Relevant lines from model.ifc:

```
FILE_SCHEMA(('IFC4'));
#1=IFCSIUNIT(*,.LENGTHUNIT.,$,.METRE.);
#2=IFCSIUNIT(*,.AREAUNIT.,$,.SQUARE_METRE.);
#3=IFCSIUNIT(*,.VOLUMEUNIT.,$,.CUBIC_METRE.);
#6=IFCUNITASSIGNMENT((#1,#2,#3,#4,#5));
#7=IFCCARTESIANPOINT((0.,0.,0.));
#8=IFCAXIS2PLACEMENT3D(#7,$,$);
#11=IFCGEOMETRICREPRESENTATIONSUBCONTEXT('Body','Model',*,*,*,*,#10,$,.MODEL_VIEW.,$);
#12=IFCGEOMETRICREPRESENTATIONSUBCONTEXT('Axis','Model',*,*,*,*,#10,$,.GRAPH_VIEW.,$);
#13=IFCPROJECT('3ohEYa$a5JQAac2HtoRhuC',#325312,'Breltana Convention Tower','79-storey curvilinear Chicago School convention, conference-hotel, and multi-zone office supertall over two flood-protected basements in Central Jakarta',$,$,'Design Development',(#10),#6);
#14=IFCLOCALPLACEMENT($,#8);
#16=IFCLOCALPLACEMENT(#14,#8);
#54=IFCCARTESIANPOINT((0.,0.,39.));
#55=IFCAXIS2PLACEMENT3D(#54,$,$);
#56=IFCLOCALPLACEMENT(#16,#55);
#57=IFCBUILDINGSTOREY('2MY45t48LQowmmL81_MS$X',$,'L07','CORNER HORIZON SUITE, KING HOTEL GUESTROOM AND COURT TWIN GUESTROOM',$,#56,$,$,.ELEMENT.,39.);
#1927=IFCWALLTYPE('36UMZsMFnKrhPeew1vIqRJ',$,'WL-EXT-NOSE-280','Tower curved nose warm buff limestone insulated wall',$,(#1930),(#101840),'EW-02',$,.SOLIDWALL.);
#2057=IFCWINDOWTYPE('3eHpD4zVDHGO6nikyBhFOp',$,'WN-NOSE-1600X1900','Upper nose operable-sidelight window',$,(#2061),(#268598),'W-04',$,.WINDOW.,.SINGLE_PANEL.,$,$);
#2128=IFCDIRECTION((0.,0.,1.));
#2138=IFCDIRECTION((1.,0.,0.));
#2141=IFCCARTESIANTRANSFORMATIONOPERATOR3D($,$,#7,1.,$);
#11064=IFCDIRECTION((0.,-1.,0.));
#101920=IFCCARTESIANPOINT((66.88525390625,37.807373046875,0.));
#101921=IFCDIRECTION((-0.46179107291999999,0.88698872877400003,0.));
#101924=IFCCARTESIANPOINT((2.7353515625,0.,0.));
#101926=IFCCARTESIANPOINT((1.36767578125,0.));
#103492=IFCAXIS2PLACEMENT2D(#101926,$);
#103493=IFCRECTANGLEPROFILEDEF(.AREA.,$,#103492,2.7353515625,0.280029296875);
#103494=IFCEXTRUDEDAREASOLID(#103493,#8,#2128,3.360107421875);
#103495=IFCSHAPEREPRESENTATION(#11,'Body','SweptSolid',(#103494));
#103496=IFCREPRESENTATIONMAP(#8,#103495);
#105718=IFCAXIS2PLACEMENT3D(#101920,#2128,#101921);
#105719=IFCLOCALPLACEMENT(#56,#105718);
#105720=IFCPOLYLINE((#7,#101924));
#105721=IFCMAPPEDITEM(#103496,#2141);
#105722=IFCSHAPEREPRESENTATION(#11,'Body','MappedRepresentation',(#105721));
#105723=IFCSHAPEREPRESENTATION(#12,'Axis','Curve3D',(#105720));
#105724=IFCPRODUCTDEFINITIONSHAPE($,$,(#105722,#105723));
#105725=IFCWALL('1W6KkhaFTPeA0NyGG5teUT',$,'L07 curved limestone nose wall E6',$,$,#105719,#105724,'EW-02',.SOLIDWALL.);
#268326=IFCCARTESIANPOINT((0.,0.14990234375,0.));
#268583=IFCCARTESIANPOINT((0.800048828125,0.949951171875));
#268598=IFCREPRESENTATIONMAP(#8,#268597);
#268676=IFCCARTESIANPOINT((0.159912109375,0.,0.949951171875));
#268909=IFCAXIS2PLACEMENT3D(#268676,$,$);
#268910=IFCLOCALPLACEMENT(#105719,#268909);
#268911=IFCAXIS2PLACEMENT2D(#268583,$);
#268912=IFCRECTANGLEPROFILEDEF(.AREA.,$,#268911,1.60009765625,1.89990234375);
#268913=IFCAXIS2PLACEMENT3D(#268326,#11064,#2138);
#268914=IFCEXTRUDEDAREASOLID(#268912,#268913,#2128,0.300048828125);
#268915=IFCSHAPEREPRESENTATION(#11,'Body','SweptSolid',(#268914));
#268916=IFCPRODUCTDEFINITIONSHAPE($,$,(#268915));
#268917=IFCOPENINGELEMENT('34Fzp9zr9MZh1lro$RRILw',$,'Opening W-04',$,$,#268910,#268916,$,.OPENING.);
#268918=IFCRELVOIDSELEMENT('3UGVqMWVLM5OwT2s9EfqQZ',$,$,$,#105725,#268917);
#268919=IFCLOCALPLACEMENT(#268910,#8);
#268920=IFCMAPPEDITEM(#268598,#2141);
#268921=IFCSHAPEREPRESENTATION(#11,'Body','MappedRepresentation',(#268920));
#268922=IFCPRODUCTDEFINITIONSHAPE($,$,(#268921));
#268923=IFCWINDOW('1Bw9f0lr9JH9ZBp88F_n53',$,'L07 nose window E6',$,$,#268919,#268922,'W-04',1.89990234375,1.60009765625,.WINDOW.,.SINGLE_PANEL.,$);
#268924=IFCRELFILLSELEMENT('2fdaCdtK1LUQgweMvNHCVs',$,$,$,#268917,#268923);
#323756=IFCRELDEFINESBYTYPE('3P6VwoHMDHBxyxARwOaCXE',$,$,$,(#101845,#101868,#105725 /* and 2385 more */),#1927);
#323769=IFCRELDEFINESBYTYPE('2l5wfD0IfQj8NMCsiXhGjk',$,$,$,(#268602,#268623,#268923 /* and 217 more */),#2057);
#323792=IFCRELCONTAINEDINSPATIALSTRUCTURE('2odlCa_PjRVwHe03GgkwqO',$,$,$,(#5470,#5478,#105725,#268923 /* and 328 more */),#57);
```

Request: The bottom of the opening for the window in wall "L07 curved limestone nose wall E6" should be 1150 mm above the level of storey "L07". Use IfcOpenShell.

```python
import numpy as np
import ifcopenshell
import ifcopenshell.api.geometry
import ifcopenshell.geom
import ifcopenshell.util.element
import ifcopenshell.util.placement
import ifcopenshell.util.shape
import ifcopenshell.util.unit

model = ifcopenshell.open("model.ifc")
unit_scale = ifcopenshell.util.unit.calculate_unit_scale(model)

window = model.by_guid("1Bw9f0lr9JH9ZBp88F_n53")
opening = window.FillsVoids[0].RelatingOpeningElement
storey = ifcopenshell.util.element.get_container(window, ifc_class="IfcBuildingStorey")
level = ifcopenshell.util.placement.get_local_placement(storey.ObjectPlacement)[2, 3]

# The opening's origin need not be at the sill, so measure its lowest point.
shape = ifcopenshell.geom.create_shape(ifcopenshell.geom.settings(), opening)
bottom = ifcopenshell.util.shape.get_shape_bottom_elevation(shape, shape.geometry) / unit_scale
dz = level + 1.15 / unit_scale - bottom

shift = np.array([0.0, 0.0, dz])
# The window is placed relative to its opening, so it follows when the opening moves.
matrix = ifcopenshell.util.placement.get_local_placement(opening.ObjectPlacement)
matrix[:3, 3] += shift
ifcopenshell.api.geometry.edit_object_placement(
    model, product=opening, matrix=matrix, is_si=False, should_transform_children=True
)

print(f"moved by {dz * unit_scale:+.3f} m")

model.write("model_updated.ifc")
```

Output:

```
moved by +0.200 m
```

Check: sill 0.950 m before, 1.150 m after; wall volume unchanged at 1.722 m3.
